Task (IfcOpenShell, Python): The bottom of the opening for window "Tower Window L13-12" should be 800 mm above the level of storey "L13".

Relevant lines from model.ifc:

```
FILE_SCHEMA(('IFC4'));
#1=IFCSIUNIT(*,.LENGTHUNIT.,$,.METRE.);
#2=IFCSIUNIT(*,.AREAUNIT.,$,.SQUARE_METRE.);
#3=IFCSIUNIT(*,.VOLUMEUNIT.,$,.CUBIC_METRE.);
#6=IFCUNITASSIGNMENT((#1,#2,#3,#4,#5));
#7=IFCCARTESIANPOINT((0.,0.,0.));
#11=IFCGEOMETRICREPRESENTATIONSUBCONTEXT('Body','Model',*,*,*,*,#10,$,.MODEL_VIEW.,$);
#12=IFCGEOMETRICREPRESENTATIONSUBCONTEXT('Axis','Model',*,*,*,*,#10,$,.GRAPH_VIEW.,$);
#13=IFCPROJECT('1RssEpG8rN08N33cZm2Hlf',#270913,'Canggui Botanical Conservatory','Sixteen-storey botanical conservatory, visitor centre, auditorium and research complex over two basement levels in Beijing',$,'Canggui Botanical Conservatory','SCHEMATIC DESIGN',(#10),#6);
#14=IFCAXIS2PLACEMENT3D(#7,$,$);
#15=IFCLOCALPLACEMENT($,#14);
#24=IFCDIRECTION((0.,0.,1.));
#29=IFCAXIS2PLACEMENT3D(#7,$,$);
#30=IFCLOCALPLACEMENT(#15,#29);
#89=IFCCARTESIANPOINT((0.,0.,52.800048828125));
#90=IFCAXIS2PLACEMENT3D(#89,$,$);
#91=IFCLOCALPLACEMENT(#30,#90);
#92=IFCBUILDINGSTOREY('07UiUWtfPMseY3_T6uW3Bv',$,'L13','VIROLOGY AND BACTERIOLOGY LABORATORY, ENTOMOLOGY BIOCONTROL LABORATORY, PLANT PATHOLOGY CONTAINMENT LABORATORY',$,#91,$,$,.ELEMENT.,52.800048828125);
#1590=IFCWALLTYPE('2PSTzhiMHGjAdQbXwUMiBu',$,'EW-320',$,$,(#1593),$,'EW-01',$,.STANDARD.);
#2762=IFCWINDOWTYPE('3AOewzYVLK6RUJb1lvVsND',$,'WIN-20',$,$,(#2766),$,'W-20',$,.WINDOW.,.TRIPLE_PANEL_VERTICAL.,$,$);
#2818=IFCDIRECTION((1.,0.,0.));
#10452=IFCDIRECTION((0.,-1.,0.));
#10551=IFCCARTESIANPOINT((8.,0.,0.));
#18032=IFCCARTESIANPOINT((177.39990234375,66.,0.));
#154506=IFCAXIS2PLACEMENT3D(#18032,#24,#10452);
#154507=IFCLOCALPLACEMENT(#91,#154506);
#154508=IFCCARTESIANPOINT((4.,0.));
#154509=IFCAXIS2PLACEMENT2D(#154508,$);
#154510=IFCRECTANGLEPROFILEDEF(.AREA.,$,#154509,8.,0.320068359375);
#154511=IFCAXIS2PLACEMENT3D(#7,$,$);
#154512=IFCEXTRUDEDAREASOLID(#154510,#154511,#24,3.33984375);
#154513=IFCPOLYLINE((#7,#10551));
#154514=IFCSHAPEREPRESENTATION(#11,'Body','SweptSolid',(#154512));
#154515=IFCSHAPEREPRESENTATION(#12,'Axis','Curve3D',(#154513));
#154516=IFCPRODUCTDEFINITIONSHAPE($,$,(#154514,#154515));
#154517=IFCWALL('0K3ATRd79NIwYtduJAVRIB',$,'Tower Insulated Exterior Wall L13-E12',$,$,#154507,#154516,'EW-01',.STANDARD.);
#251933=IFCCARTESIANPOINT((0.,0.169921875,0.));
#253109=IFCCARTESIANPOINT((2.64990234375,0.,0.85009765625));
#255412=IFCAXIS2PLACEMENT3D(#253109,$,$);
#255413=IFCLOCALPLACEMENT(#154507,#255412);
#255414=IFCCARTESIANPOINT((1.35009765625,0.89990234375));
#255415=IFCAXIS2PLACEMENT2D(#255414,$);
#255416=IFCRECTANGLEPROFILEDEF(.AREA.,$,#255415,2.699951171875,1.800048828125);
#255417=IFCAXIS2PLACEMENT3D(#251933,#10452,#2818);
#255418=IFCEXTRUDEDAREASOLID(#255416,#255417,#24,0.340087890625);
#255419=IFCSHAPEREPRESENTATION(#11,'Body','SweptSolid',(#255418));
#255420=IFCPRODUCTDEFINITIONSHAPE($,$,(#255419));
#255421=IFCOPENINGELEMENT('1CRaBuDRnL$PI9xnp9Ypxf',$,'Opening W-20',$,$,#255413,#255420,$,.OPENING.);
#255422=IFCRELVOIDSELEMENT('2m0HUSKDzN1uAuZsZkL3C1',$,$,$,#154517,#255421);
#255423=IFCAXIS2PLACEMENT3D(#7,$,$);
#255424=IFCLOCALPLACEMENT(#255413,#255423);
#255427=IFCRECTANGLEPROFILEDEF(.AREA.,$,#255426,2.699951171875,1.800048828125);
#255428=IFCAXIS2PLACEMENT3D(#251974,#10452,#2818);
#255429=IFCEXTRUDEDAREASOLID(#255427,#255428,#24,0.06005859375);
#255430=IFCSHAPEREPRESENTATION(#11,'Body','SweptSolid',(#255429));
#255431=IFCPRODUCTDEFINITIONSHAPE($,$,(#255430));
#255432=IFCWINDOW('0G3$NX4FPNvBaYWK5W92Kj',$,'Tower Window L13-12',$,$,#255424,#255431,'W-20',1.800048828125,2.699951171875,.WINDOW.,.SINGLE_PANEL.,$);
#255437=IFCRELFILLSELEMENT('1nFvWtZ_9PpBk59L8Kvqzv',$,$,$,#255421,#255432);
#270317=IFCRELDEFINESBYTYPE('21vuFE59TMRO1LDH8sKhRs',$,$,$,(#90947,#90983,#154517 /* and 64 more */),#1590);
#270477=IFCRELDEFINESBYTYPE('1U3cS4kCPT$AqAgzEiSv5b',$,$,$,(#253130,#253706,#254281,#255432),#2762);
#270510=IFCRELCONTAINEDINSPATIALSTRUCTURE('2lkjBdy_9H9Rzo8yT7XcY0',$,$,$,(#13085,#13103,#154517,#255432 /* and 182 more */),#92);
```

```python
import numpy as np
import ifcopenshell
import ifcopenshell.api.geometry
import ifcopenshell.geom
import ifcopenshell.util.element
import ifcopenshell.util.placement
import ifcopenshell.util.shape
import ifcopenshell.util.unit

model = ifcopenshell.open("model.ifc")
unit_scale = ifcopenshell.util.unit.calculate_unit_scale(model)

window = model.by_id(255432)
opening = window.FillsVoids[0].RelatingOpeningElement
storey = ifcopenshell.util.element.get_container(window, ifc_class="IfcBuildingStorey")
level = ifcopenshell.util.placement.get_local_placement(storey.ObjectPlacement)[2, 3]

# The opening's origin need not be at the sill, so measure its lowest point.
shape = ifcopenshell.geom.create_shape(ifcopenshell.geom.settings(), opening)
bottom = ifcopenshell.util.shape.get_shape_bottom_elevation(shape, shape.geometry) / unit_scale
dz = level + 0.8 - bottom

shift = np.array([0.0, 0.0, dz])
# The window is placed relative to its opening, so it follows when the opening moves.
matrix = ifcopenshell.util.placement.get_local_placement(opening.ObjectPlacement)
matrix[:3, 3] += shift
ifcopenshell.api.geometry.edit_object_placement(
    model, product=opening, matrix=matrix, is_si=False, should_transform_children=True
)

print(f"moved by {dz * unit_scale:+.3f} m")

model.write("model_rev.ifc")
```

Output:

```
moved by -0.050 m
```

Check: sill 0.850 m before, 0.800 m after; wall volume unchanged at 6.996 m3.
